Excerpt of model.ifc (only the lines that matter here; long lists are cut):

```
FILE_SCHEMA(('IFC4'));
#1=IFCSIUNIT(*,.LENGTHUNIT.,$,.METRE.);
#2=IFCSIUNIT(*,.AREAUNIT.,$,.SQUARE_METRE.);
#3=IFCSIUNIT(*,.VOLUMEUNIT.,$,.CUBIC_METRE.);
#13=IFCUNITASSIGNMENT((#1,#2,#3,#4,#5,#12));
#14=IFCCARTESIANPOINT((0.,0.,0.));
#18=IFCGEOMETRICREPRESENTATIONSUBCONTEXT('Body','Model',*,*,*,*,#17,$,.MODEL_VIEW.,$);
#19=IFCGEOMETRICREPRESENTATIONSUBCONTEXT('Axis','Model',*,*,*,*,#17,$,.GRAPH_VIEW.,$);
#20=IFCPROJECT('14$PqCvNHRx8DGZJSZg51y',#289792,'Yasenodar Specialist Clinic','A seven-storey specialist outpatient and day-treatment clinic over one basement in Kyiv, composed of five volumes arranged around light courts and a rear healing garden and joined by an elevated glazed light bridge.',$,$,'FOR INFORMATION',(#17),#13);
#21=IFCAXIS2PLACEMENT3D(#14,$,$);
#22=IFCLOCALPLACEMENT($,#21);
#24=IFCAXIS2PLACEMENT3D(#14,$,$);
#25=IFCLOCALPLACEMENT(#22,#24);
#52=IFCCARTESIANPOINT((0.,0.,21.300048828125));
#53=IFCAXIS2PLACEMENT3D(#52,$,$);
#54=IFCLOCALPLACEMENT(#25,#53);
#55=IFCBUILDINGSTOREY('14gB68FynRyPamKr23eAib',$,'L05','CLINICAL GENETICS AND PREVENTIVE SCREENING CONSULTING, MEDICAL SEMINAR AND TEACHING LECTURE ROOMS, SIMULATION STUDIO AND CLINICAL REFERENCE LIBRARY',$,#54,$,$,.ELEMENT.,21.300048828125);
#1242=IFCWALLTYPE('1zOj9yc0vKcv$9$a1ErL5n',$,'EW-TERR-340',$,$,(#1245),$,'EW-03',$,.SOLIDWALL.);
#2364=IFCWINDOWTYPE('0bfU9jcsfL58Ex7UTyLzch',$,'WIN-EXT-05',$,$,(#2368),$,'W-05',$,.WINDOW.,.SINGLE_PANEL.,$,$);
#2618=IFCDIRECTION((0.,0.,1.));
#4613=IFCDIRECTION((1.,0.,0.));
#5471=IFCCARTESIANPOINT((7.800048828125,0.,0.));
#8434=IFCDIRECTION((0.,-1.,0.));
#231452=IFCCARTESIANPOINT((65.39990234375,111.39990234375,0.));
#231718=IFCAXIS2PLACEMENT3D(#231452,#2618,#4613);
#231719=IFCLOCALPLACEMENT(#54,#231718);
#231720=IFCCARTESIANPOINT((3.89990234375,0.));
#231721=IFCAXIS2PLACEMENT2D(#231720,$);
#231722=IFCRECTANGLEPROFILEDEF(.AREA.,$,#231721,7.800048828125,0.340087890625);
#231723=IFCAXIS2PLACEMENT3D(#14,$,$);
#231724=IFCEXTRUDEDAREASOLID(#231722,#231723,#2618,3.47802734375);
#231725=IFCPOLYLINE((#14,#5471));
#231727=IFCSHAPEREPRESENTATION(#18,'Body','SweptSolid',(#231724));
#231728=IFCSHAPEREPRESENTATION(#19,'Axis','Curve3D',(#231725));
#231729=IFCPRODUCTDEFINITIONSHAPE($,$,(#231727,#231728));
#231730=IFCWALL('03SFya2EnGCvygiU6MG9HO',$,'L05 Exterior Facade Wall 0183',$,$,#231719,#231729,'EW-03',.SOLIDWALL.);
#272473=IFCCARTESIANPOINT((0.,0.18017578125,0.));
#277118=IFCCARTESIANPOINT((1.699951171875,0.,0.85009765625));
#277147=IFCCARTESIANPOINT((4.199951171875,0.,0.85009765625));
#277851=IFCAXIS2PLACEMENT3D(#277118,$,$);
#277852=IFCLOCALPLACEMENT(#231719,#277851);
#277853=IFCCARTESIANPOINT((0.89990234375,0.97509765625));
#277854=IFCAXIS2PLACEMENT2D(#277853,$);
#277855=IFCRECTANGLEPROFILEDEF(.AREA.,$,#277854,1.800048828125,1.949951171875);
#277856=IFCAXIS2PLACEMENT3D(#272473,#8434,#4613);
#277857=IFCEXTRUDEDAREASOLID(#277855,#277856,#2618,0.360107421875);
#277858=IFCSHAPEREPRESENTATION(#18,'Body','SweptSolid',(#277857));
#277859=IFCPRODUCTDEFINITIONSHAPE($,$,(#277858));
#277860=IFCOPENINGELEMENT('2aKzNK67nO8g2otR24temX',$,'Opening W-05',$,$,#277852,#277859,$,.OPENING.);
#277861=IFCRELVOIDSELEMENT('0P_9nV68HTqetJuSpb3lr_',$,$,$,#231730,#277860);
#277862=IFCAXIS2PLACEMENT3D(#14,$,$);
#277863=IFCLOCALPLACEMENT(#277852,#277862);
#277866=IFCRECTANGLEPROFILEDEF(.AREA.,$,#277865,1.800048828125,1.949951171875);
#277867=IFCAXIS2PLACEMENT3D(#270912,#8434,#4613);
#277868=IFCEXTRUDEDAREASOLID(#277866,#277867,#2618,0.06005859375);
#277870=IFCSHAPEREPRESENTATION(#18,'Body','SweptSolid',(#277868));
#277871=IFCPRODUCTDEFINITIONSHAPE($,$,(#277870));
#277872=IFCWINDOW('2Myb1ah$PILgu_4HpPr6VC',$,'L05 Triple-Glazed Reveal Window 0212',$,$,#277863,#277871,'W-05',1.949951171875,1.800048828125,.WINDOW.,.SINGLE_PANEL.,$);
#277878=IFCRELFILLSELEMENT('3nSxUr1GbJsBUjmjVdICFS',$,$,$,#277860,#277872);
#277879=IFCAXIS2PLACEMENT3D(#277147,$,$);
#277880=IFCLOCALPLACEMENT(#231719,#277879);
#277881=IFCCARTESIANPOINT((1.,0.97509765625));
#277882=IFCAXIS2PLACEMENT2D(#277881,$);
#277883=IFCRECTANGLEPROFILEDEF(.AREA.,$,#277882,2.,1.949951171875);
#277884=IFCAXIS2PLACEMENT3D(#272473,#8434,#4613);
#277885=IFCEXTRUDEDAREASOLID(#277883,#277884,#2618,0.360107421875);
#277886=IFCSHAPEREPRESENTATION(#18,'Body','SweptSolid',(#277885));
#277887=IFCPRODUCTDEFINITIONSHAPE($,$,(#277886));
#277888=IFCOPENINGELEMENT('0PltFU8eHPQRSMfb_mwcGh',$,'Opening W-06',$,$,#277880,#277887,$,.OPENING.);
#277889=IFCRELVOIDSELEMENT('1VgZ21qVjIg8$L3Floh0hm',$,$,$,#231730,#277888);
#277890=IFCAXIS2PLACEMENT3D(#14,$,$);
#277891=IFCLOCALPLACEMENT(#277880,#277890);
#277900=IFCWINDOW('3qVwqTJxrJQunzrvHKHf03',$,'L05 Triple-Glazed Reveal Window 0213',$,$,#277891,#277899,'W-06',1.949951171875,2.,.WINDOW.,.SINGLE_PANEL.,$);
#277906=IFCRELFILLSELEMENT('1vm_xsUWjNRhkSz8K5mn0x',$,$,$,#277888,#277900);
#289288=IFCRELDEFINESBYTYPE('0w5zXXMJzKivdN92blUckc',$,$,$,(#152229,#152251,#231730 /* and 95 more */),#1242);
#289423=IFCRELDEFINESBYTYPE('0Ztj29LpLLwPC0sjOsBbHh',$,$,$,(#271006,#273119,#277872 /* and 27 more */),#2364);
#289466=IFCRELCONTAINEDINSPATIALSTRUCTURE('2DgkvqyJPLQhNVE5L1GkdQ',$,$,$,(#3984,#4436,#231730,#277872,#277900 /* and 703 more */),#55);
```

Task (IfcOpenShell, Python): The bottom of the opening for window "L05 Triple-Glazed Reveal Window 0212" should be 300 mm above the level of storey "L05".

```python
import numpy as np
import ifcopenshell
import ifcopenshell.api.geometry
import ifcopenshell.geom
import ifcopenshell.util.element
import ifcopenshell.util.placement
import ifcopenshell.util.shape
import ifcopenshell.util.unit

model = ifcopenshell.open("model.ifc")
unit_scale = ifcopenshell.util.unit.calculate_unit_scale(model)

window = model.by_id(277872)
opening = window.FillsVoids[0].RelatingOpeningElement
storey = ifcopenshell.util.element.get_container(window, ifc_class="IfcBuildingStorey")
level = ifcopenshell.util.placement.get_local_placement(storey.ObjectPlacement)[2, 3]

# The opening's origin need not be at the sill, so measure its lowest point.
shape = ifcopenshell.geom.create_shape(ifcopenshell.geom.settings(), opening)
bottom = ifcopenshell.util.shape.get_shape_bottom_elevation(shape, shape.geometry) / unit_scale
dz = level + 0.3 / unit_scale - bottom

shift = np.array([0.0, 0.0, dz])
# The window is placed relative to its opening, so it follows when the opening moves.
matrix = ifcopenshell.util.placement.get_local_placement(opening.ObjectPlacement)
matrix[:3, 3] += shift
ifcopenshell.api.geometry.edit_object_placement(
    model, product=opening, matrix=matrix, is_si=False, should_transform_children=True
)

print(f"moved by {dz * unit_scale:+.3f} m")

model.write("model_updated.ifc")
```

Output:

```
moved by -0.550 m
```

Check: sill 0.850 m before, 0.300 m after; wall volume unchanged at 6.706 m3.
